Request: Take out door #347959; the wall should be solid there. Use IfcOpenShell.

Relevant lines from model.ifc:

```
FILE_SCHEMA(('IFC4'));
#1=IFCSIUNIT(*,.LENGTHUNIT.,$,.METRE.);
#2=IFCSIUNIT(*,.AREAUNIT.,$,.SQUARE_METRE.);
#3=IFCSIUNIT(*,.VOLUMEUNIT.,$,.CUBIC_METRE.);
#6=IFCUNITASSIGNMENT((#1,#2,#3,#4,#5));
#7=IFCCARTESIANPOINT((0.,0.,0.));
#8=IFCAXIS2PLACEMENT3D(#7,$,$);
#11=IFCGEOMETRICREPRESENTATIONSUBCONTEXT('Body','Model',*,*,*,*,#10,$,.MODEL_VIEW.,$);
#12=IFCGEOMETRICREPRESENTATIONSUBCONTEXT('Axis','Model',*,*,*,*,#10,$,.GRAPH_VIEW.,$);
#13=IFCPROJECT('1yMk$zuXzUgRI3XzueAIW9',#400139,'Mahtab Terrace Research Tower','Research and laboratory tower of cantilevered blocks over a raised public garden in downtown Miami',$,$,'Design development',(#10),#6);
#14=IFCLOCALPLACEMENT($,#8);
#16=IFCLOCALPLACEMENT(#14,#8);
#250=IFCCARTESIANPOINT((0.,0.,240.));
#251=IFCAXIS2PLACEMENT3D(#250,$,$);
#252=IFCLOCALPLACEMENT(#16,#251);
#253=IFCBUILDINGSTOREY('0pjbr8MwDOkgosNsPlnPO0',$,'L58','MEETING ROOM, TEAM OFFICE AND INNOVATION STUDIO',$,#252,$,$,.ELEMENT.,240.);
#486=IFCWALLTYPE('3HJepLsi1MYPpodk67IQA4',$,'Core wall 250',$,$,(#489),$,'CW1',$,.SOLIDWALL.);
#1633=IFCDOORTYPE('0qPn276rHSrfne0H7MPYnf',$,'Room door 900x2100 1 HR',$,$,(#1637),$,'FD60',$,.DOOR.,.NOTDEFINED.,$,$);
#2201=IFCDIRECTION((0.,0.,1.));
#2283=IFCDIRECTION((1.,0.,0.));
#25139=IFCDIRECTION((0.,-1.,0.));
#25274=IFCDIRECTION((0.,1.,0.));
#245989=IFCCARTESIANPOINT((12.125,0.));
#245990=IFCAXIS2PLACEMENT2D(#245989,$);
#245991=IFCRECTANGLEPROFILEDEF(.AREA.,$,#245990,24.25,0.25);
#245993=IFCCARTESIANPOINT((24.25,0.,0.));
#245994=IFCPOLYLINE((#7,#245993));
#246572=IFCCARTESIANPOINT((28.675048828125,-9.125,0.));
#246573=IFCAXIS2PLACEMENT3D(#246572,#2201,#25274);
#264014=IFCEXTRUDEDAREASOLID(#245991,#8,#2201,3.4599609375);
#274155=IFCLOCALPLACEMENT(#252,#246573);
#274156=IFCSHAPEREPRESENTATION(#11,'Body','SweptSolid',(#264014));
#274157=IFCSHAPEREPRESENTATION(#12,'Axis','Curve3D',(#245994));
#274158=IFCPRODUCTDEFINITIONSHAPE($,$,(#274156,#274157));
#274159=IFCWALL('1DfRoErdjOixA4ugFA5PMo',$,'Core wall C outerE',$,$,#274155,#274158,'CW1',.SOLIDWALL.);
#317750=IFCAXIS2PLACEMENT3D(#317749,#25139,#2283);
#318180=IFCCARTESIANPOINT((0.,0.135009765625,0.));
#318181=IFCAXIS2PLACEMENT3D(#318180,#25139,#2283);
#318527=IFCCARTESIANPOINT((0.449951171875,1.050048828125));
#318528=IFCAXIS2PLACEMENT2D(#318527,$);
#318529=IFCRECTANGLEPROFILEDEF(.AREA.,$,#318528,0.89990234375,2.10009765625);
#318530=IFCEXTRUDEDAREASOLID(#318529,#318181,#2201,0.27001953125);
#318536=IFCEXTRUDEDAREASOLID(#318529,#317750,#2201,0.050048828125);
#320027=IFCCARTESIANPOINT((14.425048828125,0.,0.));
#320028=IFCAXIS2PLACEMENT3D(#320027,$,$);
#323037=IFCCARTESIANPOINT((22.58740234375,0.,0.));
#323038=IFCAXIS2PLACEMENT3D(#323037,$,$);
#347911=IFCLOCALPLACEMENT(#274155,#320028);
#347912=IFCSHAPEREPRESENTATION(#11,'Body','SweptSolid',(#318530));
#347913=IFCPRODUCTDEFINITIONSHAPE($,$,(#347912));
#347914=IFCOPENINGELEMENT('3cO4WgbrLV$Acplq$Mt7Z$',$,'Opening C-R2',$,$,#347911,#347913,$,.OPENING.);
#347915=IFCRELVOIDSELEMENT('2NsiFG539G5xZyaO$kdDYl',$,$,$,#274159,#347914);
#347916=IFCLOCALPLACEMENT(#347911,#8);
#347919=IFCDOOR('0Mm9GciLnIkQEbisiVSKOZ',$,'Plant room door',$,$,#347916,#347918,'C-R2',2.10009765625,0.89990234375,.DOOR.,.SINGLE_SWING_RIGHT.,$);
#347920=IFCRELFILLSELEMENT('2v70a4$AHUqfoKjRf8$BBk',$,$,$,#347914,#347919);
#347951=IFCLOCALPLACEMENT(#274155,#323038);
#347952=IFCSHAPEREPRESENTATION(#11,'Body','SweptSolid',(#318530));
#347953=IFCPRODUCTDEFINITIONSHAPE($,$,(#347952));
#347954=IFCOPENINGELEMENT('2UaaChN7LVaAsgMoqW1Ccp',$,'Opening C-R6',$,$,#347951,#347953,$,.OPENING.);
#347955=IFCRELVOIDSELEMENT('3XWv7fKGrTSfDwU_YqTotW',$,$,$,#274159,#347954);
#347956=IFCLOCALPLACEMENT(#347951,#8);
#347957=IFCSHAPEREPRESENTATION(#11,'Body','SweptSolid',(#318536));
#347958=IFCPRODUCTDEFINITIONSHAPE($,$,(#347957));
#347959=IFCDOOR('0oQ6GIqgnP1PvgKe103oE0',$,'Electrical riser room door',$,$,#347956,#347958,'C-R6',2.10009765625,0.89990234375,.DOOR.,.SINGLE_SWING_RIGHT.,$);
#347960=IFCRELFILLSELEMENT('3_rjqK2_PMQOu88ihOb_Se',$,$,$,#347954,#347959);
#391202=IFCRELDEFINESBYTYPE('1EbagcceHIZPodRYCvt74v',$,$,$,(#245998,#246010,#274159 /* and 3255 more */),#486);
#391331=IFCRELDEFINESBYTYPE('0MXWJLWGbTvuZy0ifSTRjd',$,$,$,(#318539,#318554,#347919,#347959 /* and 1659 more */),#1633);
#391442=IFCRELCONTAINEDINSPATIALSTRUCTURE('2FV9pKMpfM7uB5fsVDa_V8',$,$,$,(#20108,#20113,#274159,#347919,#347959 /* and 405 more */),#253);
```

```python
import ifcopenshell
import ifcopenshell.api.feature
import ifcopenshell.api.root
import ifcopenshell.geom
import ifcopenshell.util.shape

model = ifcopenshell.open("model.ifc")
settings = ifcopenshell.geom.settings()


def volume(element):
    """Net volume in cubic metres, openings subtracted."""
    shape = ifcopenshell.geom.create_shape(settings, element)
    return ifcopenshell.util.shape.get_volume(shape.geometry)


door = model.by_id(347959)
opening = door.FillsVoids[0].RelatingOpeningElement
wall = opening.VoidsElements[0].RelatingBuildingElement
before = volume(wall)

ifcopenshell.api.root.remove_product(model, product=door)
ifcopenshell.api.feature.remove_feature(model, feature=opening)

after = volume(wall)

print(f"wall volume {before:.3f} -> {after:.3f} m3")

model.write("model_rev.ifc")
```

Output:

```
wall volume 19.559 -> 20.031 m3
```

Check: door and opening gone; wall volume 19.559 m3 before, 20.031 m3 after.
